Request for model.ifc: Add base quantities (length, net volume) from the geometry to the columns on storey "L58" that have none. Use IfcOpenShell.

First a look at what the model holds.

```python
import ifcopenshell
import ifcopenshell.util.element
import ifcopenshell.util.unit

model = ifcopenshell.open("model.ifc")
print(model.schema)
for unit_type in ("LENGTHUNIT", "AREAUNIT", "VOLUMEUNIT"):
    print(unit_type, ifcopenshell.util.unit.calculate_unit_scale(model, unit_type))
storey = next(s for s in model.by_type("IfcBuildingStorey") if s.Name == "L58")
columns = [e for e in ifcopenshell.util.element.get_decomposition(storey) if e.is_a("IfcColumn")]
for e in sorted(columns, key=lambda e: e.id()):
    print(e.id(), e.is_a(), e.Name, list(ifcopenshell.util.element.get_psets(e, qtos_only=True)), sep=" | ")
```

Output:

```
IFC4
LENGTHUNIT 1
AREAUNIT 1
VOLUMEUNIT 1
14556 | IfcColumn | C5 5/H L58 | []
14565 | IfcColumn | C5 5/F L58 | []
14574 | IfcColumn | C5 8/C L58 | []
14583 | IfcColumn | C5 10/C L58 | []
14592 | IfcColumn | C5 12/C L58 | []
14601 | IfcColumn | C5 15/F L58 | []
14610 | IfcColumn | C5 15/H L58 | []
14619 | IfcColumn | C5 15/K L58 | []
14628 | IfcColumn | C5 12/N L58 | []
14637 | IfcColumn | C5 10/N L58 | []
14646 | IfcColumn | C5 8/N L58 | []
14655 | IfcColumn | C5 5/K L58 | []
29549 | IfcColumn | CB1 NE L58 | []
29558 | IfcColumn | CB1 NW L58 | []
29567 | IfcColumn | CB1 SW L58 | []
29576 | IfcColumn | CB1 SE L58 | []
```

```python
import ifcopenshell
import ifcopenshell.api.pset
import ifcopenshell.geom
import ifcopenshell.util.element
import ifcopenshell.util.shape
import ifcopenshell.util.unit

model = ifcopenshell.open("model.ifc")
unit_scale = ifcopenshell.util.unit.calculate_unit_scale(model)
volume_scale = ifcopenshell.util.unit.calculate_unit_scale(model, "VOLUMEUNIT")
settings = ifcopenshell.geom.settings()

storey = next(s for s in model.by_type("IfcBuildingStorey") if s.Name == "L58")
columns = [e for e in ifcopenshell.util.element.get_decomposition(storey) if e.is_a("IfcColumn")]

for e in sorted(columns, key=lambda e: e.id()):
    if ifcopenshell.util.element.get_psets(e, qtos_only=True, should_inherit=False):
        continue
    # Geometry comes back in metres, in the element's own axes.
    shape = ifcopenshell.geom.create_shape(settings, e)
    values = {
        "Length": ifcopenshell.util.shape.get_z(shape.geometry) / unit_scale,
        "NetVolume": ifcopenshell.util.shape.get_volume(shape.geometry) / volume_scale,
    }
    qto = ifcopenshell.api.pset.add_qto(model, product=e, name="Qto_ColumnBaseQuantities")
    ifcopenshell.api.pset.edit_qto(model, qto=qto, properties=values)
    print(e.id(), {k: round(v, 3) for k, v in values.items()})

model.write("model_edited.ifc")
```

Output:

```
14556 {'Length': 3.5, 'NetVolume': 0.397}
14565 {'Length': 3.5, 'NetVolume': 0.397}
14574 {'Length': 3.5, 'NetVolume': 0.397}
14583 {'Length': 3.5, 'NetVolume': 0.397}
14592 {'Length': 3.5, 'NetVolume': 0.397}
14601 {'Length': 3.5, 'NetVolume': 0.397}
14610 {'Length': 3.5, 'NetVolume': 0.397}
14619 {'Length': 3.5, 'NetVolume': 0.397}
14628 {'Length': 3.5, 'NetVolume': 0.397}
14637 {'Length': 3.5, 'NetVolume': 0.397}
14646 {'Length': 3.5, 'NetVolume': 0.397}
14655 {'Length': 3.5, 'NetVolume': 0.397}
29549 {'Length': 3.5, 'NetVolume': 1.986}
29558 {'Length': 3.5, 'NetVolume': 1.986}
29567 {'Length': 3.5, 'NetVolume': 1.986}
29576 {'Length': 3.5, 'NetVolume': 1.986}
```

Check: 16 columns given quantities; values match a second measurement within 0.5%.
